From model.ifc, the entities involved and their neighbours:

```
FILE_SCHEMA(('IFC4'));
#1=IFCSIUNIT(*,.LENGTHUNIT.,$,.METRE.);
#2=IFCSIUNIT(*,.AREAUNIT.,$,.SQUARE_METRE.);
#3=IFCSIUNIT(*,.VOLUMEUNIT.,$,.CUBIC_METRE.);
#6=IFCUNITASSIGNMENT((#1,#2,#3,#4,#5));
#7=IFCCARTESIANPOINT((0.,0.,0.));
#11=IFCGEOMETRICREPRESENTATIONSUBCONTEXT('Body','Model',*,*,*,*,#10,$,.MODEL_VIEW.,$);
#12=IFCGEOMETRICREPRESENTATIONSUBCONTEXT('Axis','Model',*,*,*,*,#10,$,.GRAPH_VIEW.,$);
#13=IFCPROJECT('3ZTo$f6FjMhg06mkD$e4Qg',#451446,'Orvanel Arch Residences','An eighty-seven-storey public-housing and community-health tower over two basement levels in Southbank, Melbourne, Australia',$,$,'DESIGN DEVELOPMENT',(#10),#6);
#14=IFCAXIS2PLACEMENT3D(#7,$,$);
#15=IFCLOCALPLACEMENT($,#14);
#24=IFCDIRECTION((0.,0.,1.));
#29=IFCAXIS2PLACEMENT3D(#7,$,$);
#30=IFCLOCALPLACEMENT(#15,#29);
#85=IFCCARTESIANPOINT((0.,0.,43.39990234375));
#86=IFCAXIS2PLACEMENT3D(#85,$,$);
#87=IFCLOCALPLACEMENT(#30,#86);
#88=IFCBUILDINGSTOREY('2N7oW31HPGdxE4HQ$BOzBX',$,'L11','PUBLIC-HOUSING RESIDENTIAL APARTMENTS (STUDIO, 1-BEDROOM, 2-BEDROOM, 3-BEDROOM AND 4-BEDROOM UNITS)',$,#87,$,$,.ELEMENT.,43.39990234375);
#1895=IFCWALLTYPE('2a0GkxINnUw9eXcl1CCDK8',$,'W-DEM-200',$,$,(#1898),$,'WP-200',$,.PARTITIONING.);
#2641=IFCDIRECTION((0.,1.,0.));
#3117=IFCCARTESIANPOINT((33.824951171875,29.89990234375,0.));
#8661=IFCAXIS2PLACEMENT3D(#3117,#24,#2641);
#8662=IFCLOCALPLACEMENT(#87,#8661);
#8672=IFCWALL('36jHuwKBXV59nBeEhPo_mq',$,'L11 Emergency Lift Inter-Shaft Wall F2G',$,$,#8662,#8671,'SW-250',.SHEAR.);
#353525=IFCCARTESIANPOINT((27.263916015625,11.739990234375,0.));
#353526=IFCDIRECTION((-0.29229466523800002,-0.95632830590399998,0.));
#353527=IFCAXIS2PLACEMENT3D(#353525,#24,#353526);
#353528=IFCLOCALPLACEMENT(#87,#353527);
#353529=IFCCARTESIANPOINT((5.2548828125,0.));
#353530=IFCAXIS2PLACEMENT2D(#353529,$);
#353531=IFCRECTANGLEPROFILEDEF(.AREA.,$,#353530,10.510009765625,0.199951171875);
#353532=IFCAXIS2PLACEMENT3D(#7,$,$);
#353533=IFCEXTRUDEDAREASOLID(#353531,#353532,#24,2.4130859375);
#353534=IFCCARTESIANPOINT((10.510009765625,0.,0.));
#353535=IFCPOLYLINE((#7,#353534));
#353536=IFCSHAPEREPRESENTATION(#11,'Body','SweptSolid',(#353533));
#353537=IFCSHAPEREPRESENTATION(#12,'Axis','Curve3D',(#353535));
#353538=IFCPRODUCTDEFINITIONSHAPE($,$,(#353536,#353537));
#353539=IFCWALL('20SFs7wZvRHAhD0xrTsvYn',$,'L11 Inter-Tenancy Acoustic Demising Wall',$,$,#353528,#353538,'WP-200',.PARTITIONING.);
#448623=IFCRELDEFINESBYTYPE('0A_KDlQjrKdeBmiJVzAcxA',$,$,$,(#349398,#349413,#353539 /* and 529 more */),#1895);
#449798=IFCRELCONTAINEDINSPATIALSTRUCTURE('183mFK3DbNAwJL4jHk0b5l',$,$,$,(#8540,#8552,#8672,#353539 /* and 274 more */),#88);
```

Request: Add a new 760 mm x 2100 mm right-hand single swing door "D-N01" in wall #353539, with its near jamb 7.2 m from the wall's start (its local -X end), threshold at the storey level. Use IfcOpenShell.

```python
import numpy as np
import ifcopenshell
import ifcopenshell.api.feature
import ifcopenshell.api.geometry
import ifcopenshell.api.root
import ifcopenshell.api.spatial
import ifcopenshell.geom
import ifcopenshell.util.element
import ifcopenshell.util.placement
import ifcopenshell.util.representation
import ifcopenshell.util.shape
import ifcopenshell.util.unit

model = ifcopenshell.open("model.ifc")
unit_scale = ifcopenshell.util.unit.calculate_unit_scale(model)
settings = ifcopenshell.geom.settings()


def volume(element):
    """Net volume in cubic metres, openings subtracted."""
    shape = ifcopenshell.geom.create_shape(settings, element)
    return ifcopenshell.util.shape.get_volume(shape.geometry)


wall = model.by_guid("20SFs7wZvRHAhD0xrTsvYn")
storey = ifcopenshell.util.element.get_container(wall, ifc_class="IfcBuildingStorey")
context = ifcopenshell.util.representation.get_context(model, "Model", "Body", "MODEL_VIEW")
before = volume(wall)

width, height, from_end, sill = 0.76, 2.1, 7.2, 0.0  # metres

# The wall runs along its own X axis, and the end named is its -X end.
wall_shape = ifcopenshell.geom.create_shape(settings, wall)
x, y, z = ifcopenshell.util.shape.get_vertices(wall_shape.geometry).T
start = x.min() + from_end
face, thickness = float(y.min()), float(y.max() - y.min())
wall_matrix = ifcopenshell.util.placement.get_local_placement(wall.ObjectPlacement)
level = ifcopenshell.util.placement.get_local_placement(storey.ObjectPlacement)[2, 3]


def in_wall(x, y):
    """Placement at x, y metres in the wall's axes, at sill height."""
    matrix = wall_matrix.copy()
    matrix[:, 3] = wall_matrix @ np.array([x / unit_scale, y / unit_scale, 0.0, 1.0])
    matrix[2, 3] = level + sill / unit_scale
    return matrix


# Opening: a box that overshoots both wall faces by 50 mm.
opening = ifcopenshell.api.root.create_entity(model, ifc_class="IfcOpeningElement", predefined_type="OPENING")
box = ifcopenshell.api.geometry.add_wall_representation(
    model, context=context, length=width, height=height, thickness=thickness + 0.1
)
ifcopenshell.api.geometry.assign_representation(model, product=opening, representation=box)
ifcopenshell.api.geometry.edit_object_placement(model, product=opening, matrix=in_wall(start, face - 0.05), is_si=False)
ifcopenshell.api.feature.add_feature(model, feature=opening, element=wall)

door = ifcopenshell.api.root.create_entity(model, ifc_class="IfcDoor", name="D-N01", predefined_type="DOOR")
door.OverallWidth, door.OverallHeight = width / unit_scale, height / unit_scale
door.OperationType = "SINGLE_SWING_RIGHT"
body = ifcopenshell.api.geometry.add_door_representation(
    model,
    context=context,
    overall_width=door.OverallWidth,
    overall_height=door.OverallHeight,
    operation_type="SINGLE_SWING_RIGHT",
    lining_properties={"LiningDepth": thickness / unit_scale, "ThresholdDepth": thickness / unit_scale},
)
ifcopenshell.api.geometry.assign_representation(model, product=door, representation=body)
ifcopenshell.api.spatial.assign_container(model, products=[door], relating_structure=storey)
ifcopenshell.api.feature.add_filling(model, opening=opening, element=door)

# The lining spans the wall, so the door starts at the wall face.
ifcopenshell.api.geometry.edit_object_placement(model, product=door, matrix=in_wall(start, face), is_si=False)

after = volume(wall)

print(f"wall volume {before:.3f} -> {after:.3f} m3")

model.write("model_updated.ifc")
```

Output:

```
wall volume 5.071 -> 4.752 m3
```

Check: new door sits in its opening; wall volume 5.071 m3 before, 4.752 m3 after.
